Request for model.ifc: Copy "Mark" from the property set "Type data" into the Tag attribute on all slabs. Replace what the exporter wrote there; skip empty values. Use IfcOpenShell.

First a look at what the model holds.

```python
import ifcopenshell
import ifcopenshell.util.element

model = ifcopenshell.open("model.ifc")
print(model.schema)
slabs = model.by_type("IfcSlab")
print(len(slabs), "slabs")
for e in slabs[:8]:
    source = ifcopenshell.util.element.get_pset(e, "Type data", "Mark")
    target = e.Tag
    print(e.id(), repr(source), repr(target), sep=" | ")
```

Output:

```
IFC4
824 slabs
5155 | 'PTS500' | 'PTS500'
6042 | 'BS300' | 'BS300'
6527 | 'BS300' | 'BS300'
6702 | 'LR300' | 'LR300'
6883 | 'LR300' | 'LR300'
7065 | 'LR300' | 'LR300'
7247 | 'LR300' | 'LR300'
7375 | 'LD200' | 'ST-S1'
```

```python
import ifcopenshell
import ifcopenshell.util.element

model = ifcopenshell.open("model.ifc")

count = 0
for e in model.by_type("IfcSlab"):
    value = ifcopenshell.util.element.get_pset(e, "Type data", "Mark")
    current = e.Tag
    if not value or not value.strip() or current == value:
        continue
    e.Tag = value
    count += 1

print(count, "slabs updated")

model.write("model_edited.ifc")
```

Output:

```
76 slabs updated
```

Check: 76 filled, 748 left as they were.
